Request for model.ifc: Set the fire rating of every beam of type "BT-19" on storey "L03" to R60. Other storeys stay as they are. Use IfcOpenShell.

First a look at what the model holds.

```python
import ifcopenshell
import ifcopenshell.util.element

model = ifcopenshell.open("model.ifc")
print(model.schema)
storey = next(s for s in model.by_type("IfcBuildingStorey") if s.Name == "L03")
beams = [e for e in ifcopenshell.util.element.get_decomposition(storey) if e.is_a("IfcBeam")]
seen = {}
for e in beams:
    element_type = ifcopenshell.util.element.get_type(e)
    key = (element_type.Name if element_type != e and element_type else None, ifcopenshell.util.element.get_pset(e, "Pset_BeamCommon", "FireRating"))
    seen[key] = seen.get(key, 0) + 1
for (name, value), count in sorted(seen.items(), key=str):
    print(count, "x", name, "|", value)
```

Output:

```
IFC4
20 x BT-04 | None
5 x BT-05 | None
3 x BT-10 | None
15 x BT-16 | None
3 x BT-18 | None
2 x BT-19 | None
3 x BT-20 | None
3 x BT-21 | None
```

```python
import ifcopenshell
import ifcopenshell.api.pset
import ifcopenshell.util.element

model = ifcopenshell.open("model.ifc")

storey = next(s for s in model.by_type("IfcBuildingStorey") if s.Name == "L03")
beams = [e for e in ifcopenshell.util.element.get_decomposition(storey) if e.is_a("IfcBeam")]

count = 0
for e in beams:
    element_type = ifcopenshell.util.element.get_type(e)
    if element_type in (None, e) or element_type.Name != "BT-19":
        continue
    # add_pset returns the element's existing set when there is one.
    pset = ifcopenshell.api.pset.add_pset(model, product=e, name="Pset_BeamCommon")
    ifcopenshell.api.pset.edit_pset(model, pset=pset, properties={"FireRating": "R60"})
    count += 1

print(count, "beams updated")

model.write("model_edited.ifc")
```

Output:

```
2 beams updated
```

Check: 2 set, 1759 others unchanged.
